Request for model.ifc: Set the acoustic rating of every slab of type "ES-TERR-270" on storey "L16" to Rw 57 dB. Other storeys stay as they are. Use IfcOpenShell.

First a look at what the model holds.

```python
import ifcopenshell
import ifcopenshell.util.element

model = ifcopenshell.open("model.ifc")
print(model.schema)
storey = next(s for s in model.by_type("IfcBuildingStorey") if s.Name == "L16")
slabs = [e for e in ifcopenshell.util.element.get_decomposition(storey) if e.is_a("IfcSlab")]
seen = {}
for e in slabs:
    element_type = ifcopenshell.util.element.get_type(e)
    key = (element_type.Name if element_type != e and element_type else None, ifcopenshell.util.element.get_pset(e, "Pset_SlabCommon", "AcousticRating"))
    seen[key] = seen.get(key, 0) + 1
for (name, value), count in sorted(seen.items(), key=str):
    print(count, "x", name, "|", value)
```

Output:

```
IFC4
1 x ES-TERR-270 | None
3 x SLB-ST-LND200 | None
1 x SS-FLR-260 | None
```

```python
import ifcopenshell
import ifcopenshell.api.pset
import ifcopenshell.util.element

model = ifcopenshell.open("model.ifc")

storey = next(s for s in model.by_type("IfcBuildingStorey") if s.Name == "L16")
slabs = [e for e in ifcopenshell.util.element.get_decomposition(storey) if e.is_a("IfcSlab")]

count = 0
for e in slabs:
    element_type = ifcopenshell.util.element.get_type(e)
    if element_type in (None, e) or element_type.Name != "ES-TERR-270":
        continue
    # add_pset returns the element's existing set when there is one.
    pset = ifcopenshell.api.pset.add_pset(model, product=e, name="Pset_SlabCommon")
    ifcopenshell.api.pset.edit_pset(model, pset=pset, properties={"AcousticRating": "Rw 57 dB"})
    count += 1

print(count, "slabs updated")

model.write("model-out.ifc")
```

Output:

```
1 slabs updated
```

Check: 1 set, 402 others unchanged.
